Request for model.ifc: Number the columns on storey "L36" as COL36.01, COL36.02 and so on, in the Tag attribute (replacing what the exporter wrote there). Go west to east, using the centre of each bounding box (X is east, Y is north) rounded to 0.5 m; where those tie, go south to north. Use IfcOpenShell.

First a look at what the model holds.

```python
import ifcopenshell
import ifcopenshell.util.element
import ifcopenshell.util.placement

model = ifcopenshell.open("model.ifc")
print(model.schema)
storey = next(s for s in model.by_type("IfcBuildingStorey") if s.Name == "L36")
columns = [e for e in ifcopenshell.util.element.get_decomposition(storey) if e.is_a("IfcColumn")]
for e in sorted(columns, key=lambda e: e.id()):
    origin = ifcopenshell.util.placement.get_local_placement(e.ObjectPlacement)[:3, 3]
    print(e.id(), e.Tag, e.Name, origin.round(2) + 0.0, sep=" | ")
```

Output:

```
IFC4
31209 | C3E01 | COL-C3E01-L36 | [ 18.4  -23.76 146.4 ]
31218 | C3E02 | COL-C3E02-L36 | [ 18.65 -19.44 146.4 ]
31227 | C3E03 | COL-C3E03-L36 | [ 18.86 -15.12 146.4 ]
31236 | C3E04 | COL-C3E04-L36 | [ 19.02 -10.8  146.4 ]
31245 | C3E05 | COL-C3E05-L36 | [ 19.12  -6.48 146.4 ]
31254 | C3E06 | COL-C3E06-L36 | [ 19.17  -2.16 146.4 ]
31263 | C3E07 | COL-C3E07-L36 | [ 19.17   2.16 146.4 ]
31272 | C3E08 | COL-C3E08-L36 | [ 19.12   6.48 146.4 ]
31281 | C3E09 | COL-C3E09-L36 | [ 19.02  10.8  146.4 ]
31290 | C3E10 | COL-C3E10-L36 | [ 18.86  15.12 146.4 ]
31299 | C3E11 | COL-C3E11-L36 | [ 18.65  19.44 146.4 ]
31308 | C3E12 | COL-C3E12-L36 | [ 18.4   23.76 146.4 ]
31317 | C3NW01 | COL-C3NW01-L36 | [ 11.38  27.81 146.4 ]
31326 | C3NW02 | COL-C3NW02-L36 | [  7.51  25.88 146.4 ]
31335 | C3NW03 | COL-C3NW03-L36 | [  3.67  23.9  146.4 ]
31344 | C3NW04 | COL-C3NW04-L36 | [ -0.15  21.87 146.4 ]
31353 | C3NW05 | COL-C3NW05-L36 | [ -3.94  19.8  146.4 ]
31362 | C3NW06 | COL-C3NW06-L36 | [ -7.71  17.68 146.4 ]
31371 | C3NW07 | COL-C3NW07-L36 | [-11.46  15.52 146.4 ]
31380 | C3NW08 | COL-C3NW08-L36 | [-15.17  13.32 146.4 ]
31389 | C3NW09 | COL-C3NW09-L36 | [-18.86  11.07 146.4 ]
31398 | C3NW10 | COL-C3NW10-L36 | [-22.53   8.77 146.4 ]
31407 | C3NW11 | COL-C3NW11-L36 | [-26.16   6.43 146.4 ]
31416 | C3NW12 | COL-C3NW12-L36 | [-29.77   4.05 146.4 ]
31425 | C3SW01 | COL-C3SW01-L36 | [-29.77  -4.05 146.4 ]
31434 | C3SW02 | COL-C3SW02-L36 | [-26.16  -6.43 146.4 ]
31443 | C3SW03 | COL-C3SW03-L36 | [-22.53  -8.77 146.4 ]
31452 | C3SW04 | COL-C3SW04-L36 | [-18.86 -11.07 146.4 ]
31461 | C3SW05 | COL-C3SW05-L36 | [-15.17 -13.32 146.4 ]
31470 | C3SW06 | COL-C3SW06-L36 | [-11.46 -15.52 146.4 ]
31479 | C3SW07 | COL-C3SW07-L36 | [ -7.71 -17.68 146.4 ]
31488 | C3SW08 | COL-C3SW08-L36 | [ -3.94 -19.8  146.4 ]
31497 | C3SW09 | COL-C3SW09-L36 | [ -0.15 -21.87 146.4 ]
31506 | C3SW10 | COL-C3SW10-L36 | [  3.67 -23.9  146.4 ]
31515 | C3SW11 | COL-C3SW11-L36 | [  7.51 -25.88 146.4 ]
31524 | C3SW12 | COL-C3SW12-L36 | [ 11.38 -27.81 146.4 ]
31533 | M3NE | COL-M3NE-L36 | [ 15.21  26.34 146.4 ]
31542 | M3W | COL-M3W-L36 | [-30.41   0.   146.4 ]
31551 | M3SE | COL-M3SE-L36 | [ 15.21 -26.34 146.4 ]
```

```python
import ifcopenshell
import ifcopenshell.geom
import ifcopenshell.util.element
import ifcopenshell.util.shape

model = ifcopenshell.open("model.ifc")
settings = ifcopenshell.geom.settings()
settings.set("use-world-coords", True)


def centre(element):
    shape = ifcopenshell.geom.create_shape(settings, element)
    return ifcopenshell.util.shape.get_bbox_centroid(shape.geometry)


storey = next(s for s in model.by_type("IfcBuildingStorey") if s.Name == "L36")
columns = [e for e in ifcopenshell.util.element.get_decomposition(storey) if e.is_a("IfcColumn")]

# Insertion points can sit at a corner or the storey origin, so sort by the geometry (in metres).
centres = {e: centre(e) for e in columns}
columns.sort(key=lambda e: (round(centres[e][0] / 0.5), centres[e][1]))

for i, e in enumerate(columns, start=1):
    number = f"COL36.{i:02d}"
    e.Tag = number
    print(e.id(), number)

model.write("model_rev.ifc")
```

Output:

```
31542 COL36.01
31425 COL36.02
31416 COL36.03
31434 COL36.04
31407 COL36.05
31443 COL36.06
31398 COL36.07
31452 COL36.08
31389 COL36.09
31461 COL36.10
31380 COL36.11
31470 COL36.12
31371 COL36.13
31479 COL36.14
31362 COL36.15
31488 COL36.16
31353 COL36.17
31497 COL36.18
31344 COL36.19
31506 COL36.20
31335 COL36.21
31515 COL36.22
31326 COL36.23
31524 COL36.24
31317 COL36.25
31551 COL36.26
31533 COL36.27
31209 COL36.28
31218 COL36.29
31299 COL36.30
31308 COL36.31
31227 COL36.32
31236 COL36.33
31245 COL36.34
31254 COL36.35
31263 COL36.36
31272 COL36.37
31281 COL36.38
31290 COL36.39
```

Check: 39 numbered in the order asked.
